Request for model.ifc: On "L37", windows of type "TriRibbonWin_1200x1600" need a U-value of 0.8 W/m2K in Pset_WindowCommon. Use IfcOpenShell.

First a look at what the model holds.

```python
import ifcopenshell
import ifcopenshell.util.element

model = ifcopenshell.open("model.ifc")
print(model.schema)
storey = next(s for s in model.by_type("IfcBuildingStorey") if s.Name == "L37")
windows = [e for e in ifcopenshell.util.element.get_decomposition(storey) if e.is_a("IfcWindow")]
seen = {}
for e in windows:
    element_type = ifcopenshell.util.element.get_type(e)
    key = (element_type.Name if element_type != e and element_type else None, ifcopenshell.util.element.get_pset(e, "Pset_WindowCommon", "ThermalTransmittance"))
    seen[key] = seen.get(key, 0) + 1
for (name, value), count in sorted(seen.items(), key=str):
    print(count, "x", name, "|", value)
```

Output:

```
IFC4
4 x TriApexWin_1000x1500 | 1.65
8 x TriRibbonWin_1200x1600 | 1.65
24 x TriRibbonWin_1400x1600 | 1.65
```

```python
import ifcopenshell
import ifcopenshell.api.pset
import ifcopenshell.util.element

model = ifcopenshell.open("model.ifc")

storey = next(s for s in model.by_type("IfcBuildingStorey") if s.Name == "L37")
windows = [e for e in ifcopenshell.util.element.get_decomposition(storey) if e.is_a("IfcWindow")]

count = 0
for e in windows:
    element_type = ifcopenshell.util.element.get_type(e)
    if element_type in (None, e) or element_type.Name != "TriRibbonWin_1200x1600":
        continue
    found = ifcopenshell.util.element.get_pset(e, "Pset_WindowCommon", should_inherit=False)
    if found:
        pset = model.by_id(found["id"])
        if len(ifcopenshell.util.element.get_elements_by_pset(pset)) > 1:
            pset = ifcopenshell.api.pset.unshare_pset(model, products=[e], pset=pset)[0]
    else:
        pset = ifcopenshell.api.pset.add_pset(model, product=e, name="Pset_WindowCommon")
    ifcopenshell.api.pset.edit_pset(model, pset=pset, properties={"ThermalTransmittance": 0.8})
    count += 1

print(count, "windows updated")

model.write("model-out.ifc")
```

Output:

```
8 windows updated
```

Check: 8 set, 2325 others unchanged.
